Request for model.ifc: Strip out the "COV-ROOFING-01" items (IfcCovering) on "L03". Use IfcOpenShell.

First a look at what the model holds.

```python
import ifcopenshell
import ifcopenshell.util.element

model = ifcopenshell.open("model.ifc")
print(model.schema)
storey = next(s for s in model.by_type("IfcBuildingStorey") if s.Name == "L03")
coverings = [e for e in ifcopenshell.util.element.get_decomposition(storey) if e.is_a("IfcCovering")]
seen = {}
for e in coverings:
    element_type = ifcopenshell.util.element.get_type(e)
    name = element_type.Name if element_type not in (None, e) else None
    seen[name] = seen.get(name, 0) + 1
for name, count in sorted(seen.items(), key=str):
    print(count, "x", name)
```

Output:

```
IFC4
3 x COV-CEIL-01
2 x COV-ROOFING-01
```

```python
import ifcopenshell
import ifcopenshell.api.root
import ifcopenshell.util.element

model = ifcopenshell.open("model.ifc")

storey = next(s for s in model.by_type("IfcBuildingStorey") if s.Name == "L03")
coverings = [e for e in ifcopenshell.util.element.get_decomposition(storey) if e.is_a("IfcCovering")]
targets = [e for e in coverings if (t := ifcopenshell.util.element.get_type(e)) not in (None, e) and t.Name == "COV-ROOFING-01"]

for e in targets:
    ifcopenshell.api.root.remove_product(model, product=e)
print(len(targets), "removed")

model.write("model-out.ifc")
```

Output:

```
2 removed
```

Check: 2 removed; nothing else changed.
